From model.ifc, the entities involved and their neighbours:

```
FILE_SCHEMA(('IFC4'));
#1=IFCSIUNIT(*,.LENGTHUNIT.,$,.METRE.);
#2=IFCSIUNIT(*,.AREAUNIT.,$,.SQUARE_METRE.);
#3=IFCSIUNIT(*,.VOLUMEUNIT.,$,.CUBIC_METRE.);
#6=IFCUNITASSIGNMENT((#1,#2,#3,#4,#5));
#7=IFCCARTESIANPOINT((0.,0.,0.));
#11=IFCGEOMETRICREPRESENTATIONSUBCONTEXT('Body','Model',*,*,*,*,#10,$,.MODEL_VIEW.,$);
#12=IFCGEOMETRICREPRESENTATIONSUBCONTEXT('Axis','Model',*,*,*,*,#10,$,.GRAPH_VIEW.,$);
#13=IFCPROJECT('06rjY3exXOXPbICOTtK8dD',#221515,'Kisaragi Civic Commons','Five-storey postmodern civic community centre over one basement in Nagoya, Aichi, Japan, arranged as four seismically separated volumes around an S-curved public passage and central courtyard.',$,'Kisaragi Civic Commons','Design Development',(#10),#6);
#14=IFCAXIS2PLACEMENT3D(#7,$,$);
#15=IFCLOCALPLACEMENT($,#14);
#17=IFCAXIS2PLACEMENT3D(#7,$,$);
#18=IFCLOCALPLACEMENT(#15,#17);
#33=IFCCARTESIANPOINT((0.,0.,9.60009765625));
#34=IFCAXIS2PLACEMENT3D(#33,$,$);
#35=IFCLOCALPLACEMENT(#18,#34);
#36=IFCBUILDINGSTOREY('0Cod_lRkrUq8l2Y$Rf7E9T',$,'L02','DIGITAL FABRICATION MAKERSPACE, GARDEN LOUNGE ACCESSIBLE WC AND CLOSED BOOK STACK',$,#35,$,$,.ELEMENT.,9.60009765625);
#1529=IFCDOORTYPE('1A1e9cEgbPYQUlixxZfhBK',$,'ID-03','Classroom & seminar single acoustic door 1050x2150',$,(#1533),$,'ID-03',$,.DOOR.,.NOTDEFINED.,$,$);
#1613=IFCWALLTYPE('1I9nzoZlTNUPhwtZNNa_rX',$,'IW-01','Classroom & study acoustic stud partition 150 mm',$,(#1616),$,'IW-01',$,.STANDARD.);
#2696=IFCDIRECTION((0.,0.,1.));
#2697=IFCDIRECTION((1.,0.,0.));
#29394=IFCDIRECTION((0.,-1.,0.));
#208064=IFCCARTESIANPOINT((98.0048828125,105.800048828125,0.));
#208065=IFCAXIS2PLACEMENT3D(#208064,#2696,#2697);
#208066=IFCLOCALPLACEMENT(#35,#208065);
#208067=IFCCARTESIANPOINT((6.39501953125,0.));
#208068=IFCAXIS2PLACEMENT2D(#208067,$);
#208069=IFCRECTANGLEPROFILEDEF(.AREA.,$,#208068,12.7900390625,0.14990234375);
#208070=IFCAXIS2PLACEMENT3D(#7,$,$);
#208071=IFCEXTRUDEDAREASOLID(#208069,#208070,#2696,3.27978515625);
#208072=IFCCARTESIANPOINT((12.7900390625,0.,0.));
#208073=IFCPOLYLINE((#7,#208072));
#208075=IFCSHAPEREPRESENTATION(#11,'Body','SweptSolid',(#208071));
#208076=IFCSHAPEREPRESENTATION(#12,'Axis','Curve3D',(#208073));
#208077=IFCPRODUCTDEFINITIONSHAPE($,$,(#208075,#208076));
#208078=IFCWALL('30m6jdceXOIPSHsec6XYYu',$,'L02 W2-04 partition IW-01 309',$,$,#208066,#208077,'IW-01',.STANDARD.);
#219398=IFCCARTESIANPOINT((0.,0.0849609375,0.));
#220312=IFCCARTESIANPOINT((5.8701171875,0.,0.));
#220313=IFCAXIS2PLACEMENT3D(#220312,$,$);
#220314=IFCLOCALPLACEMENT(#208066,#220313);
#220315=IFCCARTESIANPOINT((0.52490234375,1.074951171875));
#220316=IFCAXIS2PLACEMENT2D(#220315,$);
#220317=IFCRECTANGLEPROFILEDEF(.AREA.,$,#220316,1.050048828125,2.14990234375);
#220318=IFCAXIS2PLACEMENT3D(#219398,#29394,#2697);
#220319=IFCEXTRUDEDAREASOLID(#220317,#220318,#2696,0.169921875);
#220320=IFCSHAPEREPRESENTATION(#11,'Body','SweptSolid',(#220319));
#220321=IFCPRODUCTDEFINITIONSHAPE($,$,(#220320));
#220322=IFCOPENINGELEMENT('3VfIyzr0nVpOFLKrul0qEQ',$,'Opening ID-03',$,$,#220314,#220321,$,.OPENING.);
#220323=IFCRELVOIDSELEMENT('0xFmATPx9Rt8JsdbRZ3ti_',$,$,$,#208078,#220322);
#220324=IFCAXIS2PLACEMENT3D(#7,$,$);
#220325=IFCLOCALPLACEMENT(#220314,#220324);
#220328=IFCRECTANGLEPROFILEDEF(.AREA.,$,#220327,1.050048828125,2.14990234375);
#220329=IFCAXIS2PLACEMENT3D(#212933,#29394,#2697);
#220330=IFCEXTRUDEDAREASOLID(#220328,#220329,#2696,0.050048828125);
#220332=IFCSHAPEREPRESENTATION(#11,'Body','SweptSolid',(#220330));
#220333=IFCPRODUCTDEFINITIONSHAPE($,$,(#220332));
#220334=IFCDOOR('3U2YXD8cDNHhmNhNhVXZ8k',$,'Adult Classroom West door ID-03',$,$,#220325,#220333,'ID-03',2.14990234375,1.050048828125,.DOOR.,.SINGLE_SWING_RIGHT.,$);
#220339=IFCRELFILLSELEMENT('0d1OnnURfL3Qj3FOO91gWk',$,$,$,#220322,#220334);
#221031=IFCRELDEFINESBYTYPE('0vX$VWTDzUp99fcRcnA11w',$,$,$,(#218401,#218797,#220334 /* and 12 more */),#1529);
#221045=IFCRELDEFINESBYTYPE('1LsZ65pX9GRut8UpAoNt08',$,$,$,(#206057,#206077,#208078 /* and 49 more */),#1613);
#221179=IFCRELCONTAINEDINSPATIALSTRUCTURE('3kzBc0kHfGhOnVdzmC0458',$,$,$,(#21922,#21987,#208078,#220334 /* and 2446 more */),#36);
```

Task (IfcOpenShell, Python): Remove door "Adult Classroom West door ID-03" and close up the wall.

```python
import ifcopenshell
import ifcopenshell.api.feature
import ifcopenshell.api.root
import ifcopenshell.geom
import ifcopenshell.util.shape

model = ifcopenshell.open("model.ifc")
settings = ifcopenshell.geom.settings()


def volume(element):
    """Net volume in cubic metres, openings subtracted."""
    shape = ifcopenshell.geom.create_shape(settings, element)
    return ifcopenshell.util.shape.get_volume(shape.geometry)


door = model.by_guid("3U2YXD8cDNHhmNhNhVXZ8k")
opening = door.FillsVoids[0].RelatingOpeningElement
wall = opening.VoidsElements[0].RelatingBuildingElement
before = volume(wall)

ifcopenshell.api.root.remove_product(model, product=door)
ifcopenshell.api.feature.remove_feature(model, feature=opening)

after = volume(wall)

print(f"wall volume {before:.3f} -> {after:.3f} m3")

model.write("model_rev.ifc")
```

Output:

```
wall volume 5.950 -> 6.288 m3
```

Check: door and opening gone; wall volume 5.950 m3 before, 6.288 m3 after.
